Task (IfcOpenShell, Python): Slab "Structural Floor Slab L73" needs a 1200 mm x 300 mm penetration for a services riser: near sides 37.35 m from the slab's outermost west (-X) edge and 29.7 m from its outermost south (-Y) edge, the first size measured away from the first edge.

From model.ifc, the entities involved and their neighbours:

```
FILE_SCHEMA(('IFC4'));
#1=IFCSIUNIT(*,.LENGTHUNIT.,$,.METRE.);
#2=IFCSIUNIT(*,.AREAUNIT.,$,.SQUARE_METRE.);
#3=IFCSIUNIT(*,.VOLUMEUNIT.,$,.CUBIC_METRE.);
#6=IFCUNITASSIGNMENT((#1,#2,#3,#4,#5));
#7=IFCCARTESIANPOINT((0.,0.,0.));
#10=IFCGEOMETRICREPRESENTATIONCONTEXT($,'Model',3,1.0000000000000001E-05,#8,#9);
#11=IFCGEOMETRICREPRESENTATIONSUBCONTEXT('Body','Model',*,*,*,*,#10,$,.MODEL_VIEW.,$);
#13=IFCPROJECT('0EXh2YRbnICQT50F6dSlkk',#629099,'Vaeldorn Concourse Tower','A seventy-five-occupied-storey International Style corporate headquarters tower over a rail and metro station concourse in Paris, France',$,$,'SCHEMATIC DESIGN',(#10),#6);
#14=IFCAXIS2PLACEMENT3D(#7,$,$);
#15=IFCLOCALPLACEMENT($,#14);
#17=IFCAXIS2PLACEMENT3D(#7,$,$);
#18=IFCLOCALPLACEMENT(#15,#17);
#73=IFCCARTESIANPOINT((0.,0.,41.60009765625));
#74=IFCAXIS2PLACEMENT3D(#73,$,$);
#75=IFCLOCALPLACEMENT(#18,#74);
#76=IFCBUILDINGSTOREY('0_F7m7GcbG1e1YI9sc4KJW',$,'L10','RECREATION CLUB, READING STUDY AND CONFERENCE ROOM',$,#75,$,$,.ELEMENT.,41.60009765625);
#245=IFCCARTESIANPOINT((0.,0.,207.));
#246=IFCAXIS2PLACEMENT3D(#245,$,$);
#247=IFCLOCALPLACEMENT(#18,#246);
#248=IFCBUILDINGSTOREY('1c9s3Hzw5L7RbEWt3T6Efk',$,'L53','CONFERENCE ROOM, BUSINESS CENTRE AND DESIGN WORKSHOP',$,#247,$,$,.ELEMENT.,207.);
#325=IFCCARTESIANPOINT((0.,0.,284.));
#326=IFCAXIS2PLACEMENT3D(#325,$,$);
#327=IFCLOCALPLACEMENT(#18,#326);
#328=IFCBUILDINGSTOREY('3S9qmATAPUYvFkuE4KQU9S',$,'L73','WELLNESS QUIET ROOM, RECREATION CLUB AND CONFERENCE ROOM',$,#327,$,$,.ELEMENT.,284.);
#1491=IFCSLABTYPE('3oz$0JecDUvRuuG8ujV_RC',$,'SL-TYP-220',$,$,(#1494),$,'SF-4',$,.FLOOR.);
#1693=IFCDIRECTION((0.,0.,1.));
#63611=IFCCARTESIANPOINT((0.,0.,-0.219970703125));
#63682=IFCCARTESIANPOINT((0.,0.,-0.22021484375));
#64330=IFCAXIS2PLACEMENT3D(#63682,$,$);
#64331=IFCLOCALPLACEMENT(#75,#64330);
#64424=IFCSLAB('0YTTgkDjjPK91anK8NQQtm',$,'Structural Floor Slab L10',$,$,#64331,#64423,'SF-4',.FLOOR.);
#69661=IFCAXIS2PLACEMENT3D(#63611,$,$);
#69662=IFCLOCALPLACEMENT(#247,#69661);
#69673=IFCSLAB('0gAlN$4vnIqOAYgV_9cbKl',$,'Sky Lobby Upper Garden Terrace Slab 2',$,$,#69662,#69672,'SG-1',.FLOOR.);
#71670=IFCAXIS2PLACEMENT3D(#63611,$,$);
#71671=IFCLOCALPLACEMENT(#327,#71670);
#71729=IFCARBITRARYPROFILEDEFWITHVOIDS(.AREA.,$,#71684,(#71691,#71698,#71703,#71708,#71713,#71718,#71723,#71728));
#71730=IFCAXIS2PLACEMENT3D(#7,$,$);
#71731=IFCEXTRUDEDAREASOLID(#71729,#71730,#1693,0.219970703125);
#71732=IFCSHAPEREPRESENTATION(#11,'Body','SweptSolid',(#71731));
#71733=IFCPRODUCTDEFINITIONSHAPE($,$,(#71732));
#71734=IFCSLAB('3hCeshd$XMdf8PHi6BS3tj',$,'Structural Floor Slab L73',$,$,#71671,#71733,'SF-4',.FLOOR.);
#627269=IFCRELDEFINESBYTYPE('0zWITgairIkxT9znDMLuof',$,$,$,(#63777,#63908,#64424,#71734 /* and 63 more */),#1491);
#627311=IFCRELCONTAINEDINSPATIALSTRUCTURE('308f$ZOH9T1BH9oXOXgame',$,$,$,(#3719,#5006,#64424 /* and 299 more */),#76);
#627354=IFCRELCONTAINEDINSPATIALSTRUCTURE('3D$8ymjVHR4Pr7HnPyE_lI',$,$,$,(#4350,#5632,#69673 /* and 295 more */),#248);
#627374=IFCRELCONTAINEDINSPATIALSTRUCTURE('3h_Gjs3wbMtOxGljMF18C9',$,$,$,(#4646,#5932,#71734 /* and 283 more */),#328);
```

```python
import numpy as np
import ifcopenshell
import ifcopenshell.api.feature
import ifcopenshell.api.geometry
import ifcopenshell.api.root
import ifcopenshell.geom
import ifcopenshell.util.placement
import ifcopenshell.util.representation
import ifcopenshell.util.shape
import ifcopenshell.util.unit

model = ifcopenshell.open("model.ifc")
unit_scale = ifcopenshell.util.unit.calculate_unit_scale(model)
settings = ifcopenshell.geom.settings()


def volume(element):
    """Net volume in cubic metres, openings subtracted."""
    shape = ifcopenshell.geom.create_shape(settings, element)
    return ifcopenshell.util.shape.get_volume(shape.geometry)


slab = model.by_id(71734)
before = volume(slab)

# Extent in the slab's own axes, in metres. The edges named are its -X and -Y sides.
slab_shape = ifcopenshell.geom.create_shape(settings, slab)
vertices = ifcopenshell.util.shape.get_vertices(slab_shape.geometry)
x_min, y_min, bottom = vertices.min(axis=0)
top = vertices[:, 2].max()

opening = ifcopenshell.api.root.create_entity(model, ifc_class="IfcOpeningElement", name="Services riser opening", predefined_type="OPENING")
context = ifcopenshell.util.representation.get_context(model, "Model", "Body", "MODEL_VIEW")
width, depth = 1.2, 0.3
outline = [(0.0, 0.0), (width, 0.0), (width, depth), (0.0, depth), (0.0, 0.0)]
# Overshoot both faces by 50 mm so the cut is clean.
shape = ifcopenshell.api.geometry.add_slab_representation(
    model, context=context, depth=top - bottom + 0.1, polyline=outline
)
ifcopenshell.api.geometry.assign_representation(model, product=opening, representation=shape)

matrix = ifcopenshell.util.placement.get_local_placement(slab.ObjectPlacement)
matrix[:, 3] = matrix @ np.append(np.array([x_min + 37.35, y_min + 29.7, bottom - 0.05]) / unit_scale, 1.0)
ifcopenshell.api.geometry.edit_object_placement(model, product=opening, matrix=matrix, is_si=False)
ifcopenshell.api.feature.add_feature(model, feature=opening, element=slab)

after = volume(slab)

print(f"slab volume {before:.3f} -> {after:.3f} m3")

model.write("model_rev.ifc")
```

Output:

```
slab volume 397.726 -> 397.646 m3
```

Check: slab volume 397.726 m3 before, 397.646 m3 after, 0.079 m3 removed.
